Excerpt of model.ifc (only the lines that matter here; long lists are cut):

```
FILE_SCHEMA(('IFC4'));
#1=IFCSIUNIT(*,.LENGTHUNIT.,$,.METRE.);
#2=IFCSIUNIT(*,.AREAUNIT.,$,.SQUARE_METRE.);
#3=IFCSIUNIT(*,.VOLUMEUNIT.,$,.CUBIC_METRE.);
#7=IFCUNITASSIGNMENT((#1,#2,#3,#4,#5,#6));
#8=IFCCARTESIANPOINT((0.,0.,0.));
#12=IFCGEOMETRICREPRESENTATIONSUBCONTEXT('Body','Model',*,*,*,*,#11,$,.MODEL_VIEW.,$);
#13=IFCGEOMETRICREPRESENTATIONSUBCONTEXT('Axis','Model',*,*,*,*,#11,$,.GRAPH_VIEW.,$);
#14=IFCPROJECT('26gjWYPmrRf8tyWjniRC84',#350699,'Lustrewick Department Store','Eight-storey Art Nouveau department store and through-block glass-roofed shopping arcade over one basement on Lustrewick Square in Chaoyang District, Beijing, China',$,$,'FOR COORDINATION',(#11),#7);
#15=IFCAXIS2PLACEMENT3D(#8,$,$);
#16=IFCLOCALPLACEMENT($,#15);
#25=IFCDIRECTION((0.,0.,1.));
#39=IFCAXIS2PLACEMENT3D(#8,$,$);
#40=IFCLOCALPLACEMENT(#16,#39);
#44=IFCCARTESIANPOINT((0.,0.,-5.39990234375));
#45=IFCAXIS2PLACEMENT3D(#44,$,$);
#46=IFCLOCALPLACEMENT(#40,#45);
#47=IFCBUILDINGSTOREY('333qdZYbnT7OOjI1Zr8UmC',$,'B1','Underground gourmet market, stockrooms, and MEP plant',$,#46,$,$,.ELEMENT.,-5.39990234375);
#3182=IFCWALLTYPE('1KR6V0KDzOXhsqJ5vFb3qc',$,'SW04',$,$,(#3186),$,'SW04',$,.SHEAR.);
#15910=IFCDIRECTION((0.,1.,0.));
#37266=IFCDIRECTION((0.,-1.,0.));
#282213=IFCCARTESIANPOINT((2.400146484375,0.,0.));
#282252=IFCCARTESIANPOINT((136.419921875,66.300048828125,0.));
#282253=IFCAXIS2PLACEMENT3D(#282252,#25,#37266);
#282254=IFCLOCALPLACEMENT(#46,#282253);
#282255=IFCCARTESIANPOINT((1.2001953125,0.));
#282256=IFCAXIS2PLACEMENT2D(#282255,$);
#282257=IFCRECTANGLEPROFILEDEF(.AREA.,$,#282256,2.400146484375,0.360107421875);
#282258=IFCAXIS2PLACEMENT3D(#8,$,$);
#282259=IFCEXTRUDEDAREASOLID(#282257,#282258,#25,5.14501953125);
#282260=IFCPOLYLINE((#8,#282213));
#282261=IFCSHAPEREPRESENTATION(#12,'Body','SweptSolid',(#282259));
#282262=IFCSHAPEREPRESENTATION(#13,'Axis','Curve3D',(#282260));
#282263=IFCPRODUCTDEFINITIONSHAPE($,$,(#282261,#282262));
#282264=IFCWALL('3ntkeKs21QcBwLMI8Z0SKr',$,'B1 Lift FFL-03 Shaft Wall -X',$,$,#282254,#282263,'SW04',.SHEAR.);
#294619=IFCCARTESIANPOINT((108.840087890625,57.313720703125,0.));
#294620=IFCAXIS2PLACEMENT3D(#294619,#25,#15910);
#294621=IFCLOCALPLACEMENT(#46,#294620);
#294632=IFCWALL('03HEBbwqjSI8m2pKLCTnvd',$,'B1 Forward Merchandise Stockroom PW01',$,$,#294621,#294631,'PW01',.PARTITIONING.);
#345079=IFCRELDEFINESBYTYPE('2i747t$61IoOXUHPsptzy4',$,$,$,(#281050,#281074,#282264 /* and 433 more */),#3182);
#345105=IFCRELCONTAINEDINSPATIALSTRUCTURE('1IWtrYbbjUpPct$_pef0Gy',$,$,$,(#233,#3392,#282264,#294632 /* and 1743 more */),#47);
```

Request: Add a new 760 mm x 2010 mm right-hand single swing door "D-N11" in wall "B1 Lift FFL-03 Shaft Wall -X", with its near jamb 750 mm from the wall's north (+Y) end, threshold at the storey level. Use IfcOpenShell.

```python
import numpy as np
import ifcopenshell
import ifcopenshell.api.feature
import ifcopenshell.api.geometry
import ifcopenshell.api.root
import ifcopenshell.api.spatial
import ifcopenshell.geom
import ifcopenshell.util.element
import ifcopenshell.util.placement
import ifcopenshell.util.representation
import ifcopenshell.util.shape
import ifcopenshell.util.unit

model = ifcopenshell.open("model.ifc")
unit_scale = ifcopenshell.util.unit.calculate_unit_scale(model)
settings = ifcopenshell.geom.settings()


def volume(element):
    """Net volume in cubic metres, openings subtracted."""
    shape = ifcopenshell.geom.create_shape(settings, element)
    return ifcopenshell.util.shape.get_volume(shape.geometry)


wall = model.by_id(282264)
storey = ifcopenshell.util.element.get_container(wall, ifc_class="IfcBuildingStorey")
context = ifcopenshell.util.representation.get_context(model, "Model", "Body", "MODEL_VIEW")
before = volume(wall)

width, height, from_end, sill = 0.76, 2.01, 0.75, 0.0  # metres

# The wall runs along its own X axis, and the end named is its -X end.
wall_shape = ifcopenshell.geom.create_shape(settings, wall)
x, y, z = ifcopenshell.util.shape.get_vertices(wall_shape.geometry).T
start = x.min() + from_end
face, thickness = float(y.min()), float(y.max() - y.min())
wall_matrix = ifcopenshell.util.placement.get_local_placement(wall.ObjectPlacement)
level = ifcopenshell.util.placement.get_local_placement(storey.ObjectPlacement)[2, 3]


def in_wall(x, y):
    """Placement at x, y metres in the wall's axes, at sill height."""
    matrix = wall_matrix.copy()
    matrix[:, 3] = wall_matrix @ np.array([x / unit_scale, y / unit_scale, 0.0, 1.0])
    matrix[2, 3] = level + sill / unit_scale
    return matrix


# Opening: a box that overshoots both wall faces by 50 mm.
opening = ifcopenshell.api.root.create_entity(model, ifc_class="IfcOpeningElement", predefined_type="OPENING")
box = ifcopenshell.api.geometry.add_wall_representation(
    model, context=context, length=width, height=height, thickness=thickness + 0.1
)
ifcopenshell.api.geometry.assign_representation(model, product=opening, representation=box)
ifcopenshell.api.geometry.edit_object_placement(model, product=opening, matrix=in_wall(start, face - 0.05), is_si=False)
ifcopenshell.api.feature.add_feature(model, feature=opening, element=wall)

door = ifcopenshell.api.root.create_entity(model, ifc_class="IfcDoor", name="D-N11", predefined_type="DOOR")
door.OverallWidth, door.OverallHeight = width / unit_scale, height / unit_scale
door.OperationType = "SINGLE_SWING_RIGHT"
body = ifcopenshell.api.geometry.add_door_representation(
    model,
    context=context,
    overall_width=door.OverallWidth,
    overall_height=door.OverallHeight,
    operation_type="SINGLE_SWING_RIGHT",
    lining_properties={"LiningDepth": thickness / unit_scale, "ThresholdDepth": thickness / unit_scale},
)
ifcopenshell.api.geometry.assign_representation(model, product=door, representation=body)
ifcopenshell.api.spatial.assign_container(model, products=[door], relating_structure=storey)
ifcopenshell.api.feature.add_filling(model, opening=opening, element=door)

# The lining spans the wall, so the door starts at the wall face.
ifcopenshell.api.geometry.edit_object_placement(model, product=door, matrix=in_wall(start, face), is_si=False)

after = volume(wall)

print(f"wall volume {before:.3f} -> {after:.3f} m3")

model.write("model-out.ifc")
```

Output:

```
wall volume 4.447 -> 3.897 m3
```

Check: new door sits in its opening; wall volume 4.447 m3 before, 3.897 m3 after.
